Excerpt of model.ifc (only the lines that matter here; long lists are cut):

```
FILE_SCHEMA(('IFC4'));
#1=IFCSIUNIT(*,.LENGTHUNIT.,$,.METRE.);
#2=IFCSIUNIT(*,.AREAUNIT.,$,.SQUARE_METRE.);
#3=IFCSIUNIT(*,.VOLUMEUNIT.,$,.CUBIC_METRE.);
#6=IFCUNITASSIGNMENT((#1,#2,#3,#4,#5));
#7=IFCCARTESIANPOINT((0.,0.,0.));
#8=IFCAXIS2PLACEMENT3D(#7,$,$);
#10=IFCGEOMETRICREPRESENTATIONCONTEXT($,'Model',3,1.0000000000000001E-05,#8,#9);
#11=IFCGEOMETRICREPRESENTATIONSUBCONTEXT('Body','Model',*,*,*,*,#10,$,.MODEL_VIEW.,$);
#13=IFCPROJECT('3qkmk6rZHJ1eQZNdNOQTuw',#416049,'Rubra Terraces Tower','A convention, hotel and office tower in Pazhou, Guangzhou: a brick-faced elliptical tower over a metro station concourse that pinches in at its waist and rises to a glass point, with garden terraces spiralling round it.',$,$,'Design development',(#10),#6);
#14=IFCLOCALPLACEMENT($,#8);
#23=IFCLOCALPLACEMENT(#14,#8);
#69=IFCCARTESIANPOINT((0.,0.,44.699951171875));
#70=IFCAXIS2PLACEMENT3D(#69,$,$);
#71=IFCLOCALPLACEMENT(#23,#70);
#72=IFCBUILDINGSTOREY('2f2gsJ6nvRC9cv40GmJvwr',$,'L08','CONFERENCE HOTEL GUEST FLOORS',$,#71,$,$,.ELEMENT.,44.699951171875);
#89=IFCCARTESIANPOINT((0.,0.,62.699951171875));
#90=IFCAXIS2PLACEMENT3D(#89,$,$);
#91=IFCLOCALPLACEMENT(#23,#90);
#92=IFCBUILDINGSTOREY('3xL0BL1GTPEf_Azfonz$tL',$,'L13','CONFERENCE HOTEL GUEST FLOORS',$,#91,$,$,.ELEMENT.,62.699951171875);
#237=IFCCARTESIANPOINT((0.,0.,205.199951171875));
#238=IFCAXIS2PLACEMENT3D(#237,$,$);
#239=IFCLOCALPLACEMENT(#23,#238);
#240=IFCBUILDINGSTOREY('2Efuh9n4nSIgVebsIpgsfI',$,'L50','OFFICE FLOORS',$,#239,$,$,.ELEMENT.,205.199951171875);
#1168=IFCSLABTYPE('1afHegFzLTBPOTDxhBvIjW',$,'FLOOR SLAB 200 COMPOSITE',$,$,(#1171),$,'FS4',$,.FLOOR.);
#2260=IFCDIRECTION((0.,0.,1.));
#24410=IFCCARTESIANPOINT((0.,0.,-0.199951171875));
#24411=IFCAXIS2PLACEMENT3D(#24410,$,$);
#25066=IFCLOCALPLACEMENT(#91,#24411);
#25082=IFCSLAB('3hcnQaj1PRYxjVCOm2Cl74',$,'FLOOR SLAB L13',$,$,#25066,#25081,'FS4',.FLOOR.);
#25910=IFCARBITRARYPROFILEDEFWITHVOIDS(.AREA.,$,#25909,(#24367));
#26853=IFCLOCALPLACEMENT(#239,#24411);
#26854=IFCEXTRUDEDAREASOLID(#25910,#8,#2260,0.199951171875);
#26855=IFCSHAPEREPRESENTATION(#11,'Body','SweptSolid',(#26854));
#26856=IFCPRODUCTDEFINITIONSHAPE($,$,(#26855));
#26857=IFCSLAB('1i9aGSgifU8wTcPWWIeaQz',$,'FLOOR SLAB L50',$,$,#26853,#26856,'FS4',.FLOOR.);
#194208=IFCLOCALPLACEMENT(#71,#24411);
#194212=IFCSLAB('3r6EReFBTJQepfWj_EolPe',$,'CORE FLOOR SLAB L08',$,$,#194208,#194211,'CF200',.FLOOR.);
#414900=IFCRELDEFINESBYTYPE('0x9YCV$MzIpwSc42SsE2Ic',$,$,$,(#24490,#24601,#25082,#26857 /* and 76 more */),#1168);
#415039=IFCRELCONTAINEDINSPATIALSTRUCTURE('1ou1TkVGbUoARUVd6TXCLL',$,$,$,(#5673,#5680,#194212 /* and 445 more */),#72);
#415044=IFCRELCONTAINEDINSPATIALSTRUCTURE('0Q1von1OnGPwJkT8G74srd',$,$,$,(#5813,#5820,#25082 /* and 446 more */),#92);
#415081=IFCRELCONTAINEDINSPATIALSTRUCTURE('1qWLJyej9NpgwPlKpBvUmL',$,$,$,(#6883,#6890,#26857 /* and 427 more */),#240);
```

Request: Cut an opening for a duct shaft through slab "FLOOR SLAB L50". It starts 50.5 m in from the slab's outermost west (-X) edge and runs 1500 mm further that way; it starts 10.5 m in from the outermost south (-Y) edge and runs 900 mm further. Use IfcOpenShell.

```python
import numpy as np
import ifcopenshell
import ifcopenshell.api.feature
import ifcopenshell.api.geometry
import ifcopenshell.api.root
import ifcopenshell.geom
import ifcopenshell.util.placement
import ifcopenshell.util.representation
import ifcopenshell.util.shape
import ifcopenshell.util.unit

model = ifcopenshell.open("model.ifc")
unit_scale = ifcopenshell.util.unit.calculate_unit_scale(model)
settings = ifcopenshell.geom.settings()


def volume(element):
    """Net volume in cubic metres, openings subtracted."""
    shape = ifcopenshell.geom.create_shape(settings, element)
    return ifcopenshell.util.shape.get_volume(shape.geometry)


slab = model.by_guid("1i9aGSgifU8wTcPWWIeaQz")
before = volume(slab)

# Extent in the slab's own axes, in metres. The edges named are its -X and -Y sides.
slab_shape = ifcopenshell.geom.create_shape(settings, slab)
vertices = ifcopenshell.util.shape.get_vertices(slab_shape.geometry)
x_min, y_min, bottom = vertices.min(axis=0)
top = vertices[:, 2].max()

opening = ifcopenshell.api.root.create_entity(model, ifc_class="IfcOpeningElement", name="Duct shaft opening", predefined_type="OPENING")
context = ifcopenshell.util.representation.get_context(model, "Model", "Body", "MODEL_VIEW")
width, depth = 1.5, 0.9
outline = [(0.0, 0.0), (width, 0.0), (width, depth), (0.0, depth), (0.0, 0.0)]
# Overshoot both faces by 50 mm so the cut is clean.
shape = ifcopenshell.api.geometry.add_slab_representation(
    model, context=context, depth=top - bottom + 0.1, polyline=outline
)
ifcopenshell.api.geometry.assign_representation(model, product=opening, representation=shape)

matrix = ifcopenshell.util.placement.get_local_placement(slab.ObjectPlacement)
matrix[:, 3] = matrix @ np.append(np.array([x_min + 50.5, y_min + 10.5, bottom - 0.05]) / unit_scale, 1.0)
ifcopenshell.api.geometry.edit_object_placement(model, product=opening, matrix=matrix, is_si=False)
ifcopenshell.api.feature.add_feature(model, feature=opening, element=slab)

after = volume(slab)

print(f"slab volume {before:.3f} -> {after:.3f} m3")

model.write("model_v2.ifc")
```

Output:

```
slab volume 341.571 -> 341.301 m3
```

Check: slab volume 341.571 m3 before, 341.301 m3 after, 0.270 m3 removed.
